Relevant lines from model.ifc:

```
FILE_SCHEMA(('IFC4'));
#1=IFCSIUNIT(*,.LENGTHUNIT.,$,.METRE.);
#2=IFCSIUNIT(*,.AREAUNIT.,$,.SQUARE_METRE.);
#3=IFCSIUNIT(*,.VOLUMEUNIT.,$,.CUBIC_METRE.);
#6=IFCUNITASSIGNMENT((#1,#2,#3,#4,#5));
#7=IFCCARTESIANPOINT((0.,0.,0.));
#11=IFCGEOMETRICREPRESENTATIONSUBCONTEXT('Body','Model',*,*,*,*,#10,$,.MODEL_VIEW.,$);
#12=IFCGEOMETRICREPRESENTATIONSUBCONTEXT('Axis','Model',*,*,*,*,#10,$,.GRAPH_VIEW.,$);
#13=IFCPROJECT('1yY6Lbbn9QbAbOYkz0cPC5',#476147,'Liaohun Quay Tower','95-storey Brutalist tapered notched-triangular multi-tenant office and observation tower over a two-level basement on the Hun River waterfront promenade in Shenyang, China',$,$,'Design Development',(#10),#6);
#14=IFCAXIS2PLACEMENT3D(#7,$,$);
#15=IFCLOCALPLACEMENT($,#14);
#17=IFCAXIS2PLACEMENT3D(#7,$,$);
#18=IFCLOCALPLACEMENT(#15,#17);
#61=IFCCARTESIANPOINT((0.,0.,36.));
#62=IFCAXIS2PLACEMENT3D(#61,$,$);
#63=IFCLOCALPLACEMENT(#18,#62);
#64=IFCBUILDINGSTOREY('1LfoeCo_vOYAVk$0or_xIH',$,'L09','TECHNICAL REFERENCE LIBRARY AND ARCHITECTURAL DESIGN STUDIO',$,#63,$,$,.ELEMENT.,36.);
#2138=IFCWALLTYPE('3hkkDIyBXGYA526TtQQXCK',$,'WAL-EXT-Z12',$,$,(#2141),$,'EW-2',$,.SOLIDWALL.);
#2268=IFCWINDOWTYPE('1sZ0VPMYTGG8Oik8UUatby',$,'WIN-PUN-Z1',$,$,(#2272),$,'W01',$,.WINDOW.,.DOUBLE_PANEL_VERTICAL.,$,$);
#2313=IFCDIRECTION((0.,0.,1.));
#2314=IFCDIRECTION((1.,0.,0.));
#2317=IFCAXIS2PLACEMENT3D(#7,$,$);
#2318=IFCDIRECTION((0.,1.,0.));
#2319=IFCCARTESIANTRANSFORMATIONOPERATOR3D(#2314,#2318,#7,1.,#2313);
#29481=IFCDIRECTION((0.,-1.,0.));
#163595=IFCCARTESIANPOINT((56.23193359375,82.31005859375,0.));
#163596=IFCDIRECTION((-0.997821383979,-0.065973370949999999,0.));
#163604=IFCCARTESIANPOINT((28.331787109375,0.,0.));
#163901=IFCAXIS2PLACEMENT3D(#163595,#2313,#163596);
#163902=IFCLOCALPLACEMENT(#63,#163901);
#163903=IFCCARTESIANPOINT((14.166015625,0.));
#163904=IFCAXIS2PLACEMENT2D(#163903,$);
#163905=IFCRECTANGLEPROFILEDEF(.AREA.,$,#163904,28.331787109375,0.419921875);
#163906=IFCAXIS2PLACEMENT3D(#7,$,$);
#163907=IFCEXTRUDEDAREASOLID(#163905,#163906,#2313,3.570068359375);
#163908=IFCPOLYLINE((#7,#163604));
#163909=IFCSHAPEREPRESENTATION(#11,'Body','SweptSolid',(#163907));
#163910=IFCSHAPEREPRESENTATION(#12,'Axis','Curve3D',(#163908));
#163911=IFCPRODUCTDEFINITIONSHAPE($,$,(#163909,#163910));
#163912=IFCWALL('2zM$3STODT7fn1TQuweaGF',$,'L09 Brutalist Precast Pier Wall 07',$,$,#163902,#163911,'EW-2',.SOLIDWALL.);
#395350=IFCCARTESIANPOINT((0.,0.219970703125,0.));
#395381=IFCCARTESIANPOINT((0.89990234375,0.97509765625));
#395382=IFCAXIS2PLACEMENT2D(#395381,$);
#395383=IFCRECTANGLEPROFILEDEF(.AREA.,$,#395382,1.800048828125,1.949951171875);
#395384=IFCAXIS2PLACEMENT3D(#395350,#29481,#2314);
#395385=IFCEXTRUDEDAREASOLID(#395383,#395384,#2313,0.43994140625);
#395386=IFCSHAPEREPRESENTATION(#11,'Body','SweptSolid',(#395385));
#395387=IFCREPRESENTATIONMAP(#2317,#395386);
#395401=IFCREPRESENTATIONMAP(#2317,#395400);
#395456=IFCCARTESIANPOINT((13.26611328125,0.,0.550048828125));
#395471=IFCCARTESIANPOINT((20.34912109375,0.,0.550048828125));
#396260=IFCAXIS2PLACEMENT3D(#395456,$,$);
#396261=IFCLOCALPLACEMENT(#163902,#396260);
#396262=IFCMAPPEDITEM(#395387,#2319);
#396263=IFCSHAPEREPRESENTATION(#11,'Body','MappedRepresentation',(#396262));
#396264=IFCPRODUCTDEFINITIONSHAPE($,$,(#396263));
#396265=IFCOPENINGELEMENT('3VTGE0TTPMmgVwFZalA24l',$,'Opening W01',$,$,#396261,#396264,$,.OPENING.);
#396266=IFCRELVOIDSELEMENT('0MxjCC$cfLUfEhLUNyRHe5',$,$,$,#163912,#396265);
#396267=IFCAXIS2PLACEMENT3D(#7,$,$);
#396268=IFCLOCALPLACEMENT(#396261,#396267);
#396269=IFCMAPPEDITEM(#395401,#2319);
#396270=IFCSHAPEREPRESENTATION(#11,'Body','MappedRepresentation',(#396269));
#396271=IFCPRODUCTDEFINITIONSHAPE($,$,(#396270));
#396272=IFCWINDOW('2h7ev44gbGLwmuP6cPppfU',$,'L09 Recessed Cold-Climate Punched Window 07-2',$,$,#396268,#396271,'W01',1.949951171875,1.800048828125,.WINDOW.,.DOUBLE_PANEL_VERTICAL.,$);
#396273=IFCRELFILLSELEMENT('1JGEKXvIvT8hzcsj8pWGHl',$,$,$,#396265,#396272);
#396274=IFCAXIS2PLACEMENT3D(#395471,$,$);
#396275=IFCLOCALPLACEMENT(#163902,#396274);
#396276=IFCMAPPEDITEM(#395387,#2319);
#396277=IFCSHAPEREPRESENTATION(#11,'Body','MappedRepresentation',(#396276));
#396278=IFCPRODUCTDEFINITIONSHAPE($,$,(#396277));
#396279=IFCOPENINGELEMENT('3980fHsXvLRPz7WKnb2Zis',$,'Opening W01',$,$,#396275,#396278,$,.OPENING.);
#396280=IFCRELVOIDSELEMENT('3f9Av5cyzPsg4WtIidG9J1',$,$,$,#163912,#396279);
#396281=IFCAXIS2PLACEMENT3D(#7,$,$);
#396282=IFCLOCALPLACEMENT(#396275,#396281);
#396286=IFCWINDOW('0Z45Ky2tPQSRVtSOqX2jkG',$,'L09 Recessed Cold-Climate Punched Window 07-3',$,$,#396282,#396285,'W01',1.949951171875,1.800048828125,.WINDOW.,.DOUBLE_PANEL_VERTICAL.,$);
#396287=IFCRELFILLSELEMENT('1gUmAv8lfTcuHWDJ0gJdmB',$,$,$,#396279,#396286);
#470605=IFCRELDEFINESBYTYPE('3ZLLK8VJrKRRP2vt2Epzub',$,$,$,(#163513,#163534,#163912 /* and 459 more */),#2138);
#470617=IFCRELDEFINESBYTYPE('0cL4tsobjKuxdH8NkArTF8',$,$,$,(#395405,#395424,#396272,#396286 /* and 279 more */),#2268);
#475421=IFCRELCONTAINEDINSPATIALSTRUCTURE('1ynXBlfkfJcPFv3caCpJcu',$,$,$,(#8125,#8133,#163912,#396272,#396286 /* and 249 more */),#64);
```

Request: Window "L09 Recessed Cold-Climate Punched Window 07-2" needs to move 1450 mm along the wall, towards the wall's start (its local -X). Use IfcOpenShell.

```python
import ifcopenshell
import ifcopenshell.api.geometry
import ifcopenshell.util.placement
import ifcopenshell.util.unit

model = ifcopenshell.open("model.ifc")
unit_scale = ifcopenshell.util.unit.calculate_unit_scale(model)

window = model.by_guid("2h7ev44gbGLwmuP6cPppfU")
opening = window.FillsVoids[0].RelatingOpeningElement
wall = opening.VoidsElements[0].RelatingBuildingElement

wall_matrix = ifcopenshell.util.placement.get_local_placement(wall.ObjectPlacement)
shift = wall_matrix[:3, 0] * -1.45 / unit_scale
before = ifcopenshell.util.placement.get_local_placement(window.ObjectPlacement)[:3, 3].copy()

# The window is placed relative to its opening, so it follows when the opening moves.
matrix = ifcopenshell.util.placement.get_local_placement(opening.ObjectPlacement)
matrix[:3, 3] += shift
ifcopenshell.api.geometry.edit_object_placement(
    model, product=opening, matrix=matrix, is_si=False, should_transform_children=True
)

after = ifcopenshell.util.placement.get_local_placement(window.ObjectPlacement)[:3, 3]
print("window moved by", (after - before).round(3) + 0.0)

model.write("model_rev.ifc")
```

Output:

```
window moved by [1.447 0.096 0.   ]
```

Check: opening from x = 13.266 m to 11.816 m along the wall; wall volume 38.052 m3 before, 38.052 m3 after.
